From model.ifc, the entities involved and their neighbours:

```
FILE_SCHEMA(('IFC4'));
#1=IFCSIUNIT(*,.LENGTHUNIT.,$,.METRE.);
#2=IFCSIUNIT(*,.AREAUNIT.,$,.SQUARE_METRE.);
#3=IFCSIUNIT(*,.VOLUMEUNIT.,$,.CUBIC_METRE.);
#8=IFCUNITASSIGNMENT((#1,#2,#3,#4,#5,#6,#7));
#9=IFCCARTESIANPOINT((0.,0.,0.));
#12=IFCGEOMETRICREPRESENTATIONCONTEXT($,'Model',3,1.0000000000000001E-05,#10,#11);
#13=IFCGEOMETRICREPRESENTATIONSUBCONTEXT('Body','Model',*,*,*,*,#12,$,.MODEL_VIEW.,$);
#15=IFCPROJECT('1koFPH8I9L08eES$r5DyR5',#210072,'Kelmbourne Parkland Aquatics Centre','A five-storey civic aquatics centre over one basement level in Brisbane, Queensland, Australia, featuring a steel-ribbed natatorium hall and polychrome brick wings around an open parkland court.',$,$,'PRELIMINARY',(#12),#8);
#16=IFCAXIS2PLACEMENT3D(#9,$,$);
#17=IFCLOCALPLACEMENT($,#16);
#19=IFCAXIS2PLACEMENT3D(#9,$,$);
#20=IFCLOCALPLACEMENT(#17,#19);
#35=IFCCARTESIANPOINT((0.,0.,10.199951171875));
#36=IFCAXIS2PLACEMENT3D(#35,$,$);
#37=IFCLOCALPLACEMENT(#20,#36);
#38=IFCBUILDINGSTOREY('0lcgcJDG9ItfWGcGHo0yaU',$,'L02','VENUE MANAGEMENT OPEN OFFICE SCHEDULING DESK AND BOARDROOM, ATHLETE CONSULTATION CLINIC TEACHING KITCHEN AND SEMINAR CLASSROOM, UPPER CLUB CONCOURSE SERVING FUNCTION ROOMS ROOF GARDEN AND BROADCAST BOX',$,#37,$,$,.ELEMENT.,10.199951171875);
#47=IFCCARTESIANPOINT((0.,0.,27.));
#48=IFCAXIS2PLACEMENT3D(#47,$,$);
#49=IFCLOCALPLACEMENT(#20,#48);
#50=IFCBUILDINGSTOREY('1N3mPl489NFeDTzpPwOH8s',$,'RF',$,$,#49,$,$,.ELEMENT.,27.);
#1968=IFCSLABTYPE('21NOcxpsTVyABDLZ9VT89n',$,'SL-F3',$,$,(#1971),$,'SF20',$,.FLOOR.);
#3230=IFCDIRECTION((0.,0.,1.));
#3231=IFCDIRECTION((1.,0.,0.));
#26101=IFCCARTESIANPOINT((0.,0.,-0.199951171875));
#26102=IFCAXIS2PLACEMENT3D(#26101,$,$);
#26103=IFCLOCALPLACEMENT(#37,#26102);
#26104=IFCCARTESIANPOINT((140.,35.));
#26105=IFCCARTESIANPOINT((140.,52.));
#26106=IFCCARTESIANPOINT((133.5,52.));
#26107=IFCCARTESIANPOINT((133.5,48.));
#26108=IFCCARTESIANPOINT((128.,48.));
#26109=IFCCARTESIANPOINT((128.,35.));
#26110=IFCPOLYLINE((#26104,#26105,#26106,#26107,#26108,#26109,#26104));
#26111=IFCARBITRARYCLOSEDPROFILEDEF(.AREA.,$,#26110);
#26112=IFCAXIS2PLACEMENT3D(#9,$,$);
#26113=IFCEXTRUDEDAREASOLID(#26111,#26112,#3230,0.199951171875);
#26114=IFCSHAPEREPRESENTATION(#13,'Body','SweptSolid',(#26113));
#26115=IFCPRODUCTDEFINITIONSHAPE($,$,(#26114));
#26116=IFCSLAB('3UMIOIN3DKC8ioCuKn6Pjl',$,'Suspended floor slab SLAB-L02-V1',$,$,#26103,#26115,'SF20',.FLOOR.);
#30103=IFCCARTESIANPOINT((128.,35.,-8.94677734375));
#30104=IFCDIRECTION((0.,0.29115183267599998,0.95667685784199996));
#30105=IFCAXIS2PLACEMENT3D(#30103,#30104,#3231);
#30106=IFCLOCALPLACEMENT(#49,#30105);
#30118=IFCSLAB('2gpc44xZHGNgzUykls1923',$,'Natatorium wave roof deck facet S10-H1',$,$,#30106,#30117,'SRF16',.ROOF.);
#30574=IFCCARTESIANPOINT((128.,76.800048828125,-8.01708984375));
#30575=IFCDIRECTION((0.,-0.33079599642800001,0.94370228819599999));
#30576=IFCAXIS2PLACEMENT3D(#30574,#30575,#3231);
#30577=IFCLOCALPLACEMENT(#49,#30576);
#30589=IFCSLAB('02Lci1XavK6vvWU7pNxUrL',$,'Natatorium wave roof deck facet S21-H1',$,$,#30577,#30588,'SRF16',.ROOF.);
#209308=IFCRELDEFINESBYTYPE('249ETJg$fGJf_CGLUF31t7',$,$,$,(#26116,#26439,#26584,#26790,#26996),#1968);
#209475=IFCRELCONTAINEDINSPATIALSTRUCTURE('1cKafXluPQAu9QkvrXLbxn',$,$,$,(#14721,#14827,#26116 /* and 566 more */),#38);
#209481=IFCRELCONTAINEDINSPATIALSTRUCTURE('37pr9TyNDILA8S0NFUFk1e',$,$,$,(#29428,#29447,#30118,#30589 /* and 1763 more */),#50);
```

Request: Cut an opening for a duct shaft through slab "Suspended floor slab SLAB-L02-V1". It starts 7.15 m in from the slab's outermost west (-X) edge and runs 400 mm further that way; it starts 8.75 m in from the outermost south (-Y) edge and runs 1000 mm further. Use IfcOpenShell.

```python
import numpy as np
import ifcopenshell
import ifcopenshell.api.feature
import ifcopenshell.api.geometry
import ifcopenshell.api.root
import ifcopenshell.geom
import ifcopenshell.util.placement
import ifcopenshell.util.representation
import ifcopenshell.util.shape
import ifcopenshell.util.unit

model = ifcopenshell.open("model.ifc")
unit_scale = ifcopenshell.util.unit.calculate_unit_scale(model)
settings = ifcopenshell.geom.settings()


def volume(element):
    """Net volume in cubic metres, openings subtracted."""
    shape = ifcopenshell.geom.create_shape(settings, element)
    return ifcopenshell.util.shape.get_volume(shape.geometry)


slab = model.by_guid("3UMIOIN3DKC8ioCuKn6Pjl")
before = volume(slab)

# Extent in the slab's own axes, in metres. The edges named are its -X and -Y sides.
slab_shape = ifcopenshell.geom.create_shape(settings, slab)
vertices = ifcopenshell.util.shape.get_vertices(slab_shape.geometry)
x_min, y_min, bottom = vertices.min(axis=0)
top = vertices[:, 2].max()

opening = ifcopenshell.api.root.create_entity(model, ifc_class="IfcOpeningElement", name="Duct shaft opening", predefined_type="OPENING")
context = ifcopenshell.util.representation.get_context(model, "Model", "Body", "MODEL_VIEW")
width, depth = 0.4, 1
outline = [(0.0, 0.0), (width, 0.0), (width, depth), (0.0, depth), (0.0, 0.0)]
# Overshoot both faces by 50 mm so the cut is clean.
shape = ifcopenshell.api.geometry.add_slab_representation(
    model, context=context, depth=top - bottom + 0.1, polyline=outline
)
ifcopenshell.api.geometry.assign_representation(model, product=opening, representation=shape)

matrix = ifcopenshell.util.placement.get_local_placement(slab.ObjectPlacement)
matrix[:, 3] = matrix @ np.append(np.array([x_min + 7.15, y_min + 8.75, bottom - 0.05]) / unit_scale, 1.0)
ifcopenshell.api.geometry.edit_object_placement(model, product=opening, matrix=matrix, is_si=False)
ifcopenshell.api.feature.add_feature(model, feature=opening, element=slab)

after = volume(slab)

print(f"slab volume {before:.3f} -> {after:.3f} m3")

model.write("model-out.ifc")
```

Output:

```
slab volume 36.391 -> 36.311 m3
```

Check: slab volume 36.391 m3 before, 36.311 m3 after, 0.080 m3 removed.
